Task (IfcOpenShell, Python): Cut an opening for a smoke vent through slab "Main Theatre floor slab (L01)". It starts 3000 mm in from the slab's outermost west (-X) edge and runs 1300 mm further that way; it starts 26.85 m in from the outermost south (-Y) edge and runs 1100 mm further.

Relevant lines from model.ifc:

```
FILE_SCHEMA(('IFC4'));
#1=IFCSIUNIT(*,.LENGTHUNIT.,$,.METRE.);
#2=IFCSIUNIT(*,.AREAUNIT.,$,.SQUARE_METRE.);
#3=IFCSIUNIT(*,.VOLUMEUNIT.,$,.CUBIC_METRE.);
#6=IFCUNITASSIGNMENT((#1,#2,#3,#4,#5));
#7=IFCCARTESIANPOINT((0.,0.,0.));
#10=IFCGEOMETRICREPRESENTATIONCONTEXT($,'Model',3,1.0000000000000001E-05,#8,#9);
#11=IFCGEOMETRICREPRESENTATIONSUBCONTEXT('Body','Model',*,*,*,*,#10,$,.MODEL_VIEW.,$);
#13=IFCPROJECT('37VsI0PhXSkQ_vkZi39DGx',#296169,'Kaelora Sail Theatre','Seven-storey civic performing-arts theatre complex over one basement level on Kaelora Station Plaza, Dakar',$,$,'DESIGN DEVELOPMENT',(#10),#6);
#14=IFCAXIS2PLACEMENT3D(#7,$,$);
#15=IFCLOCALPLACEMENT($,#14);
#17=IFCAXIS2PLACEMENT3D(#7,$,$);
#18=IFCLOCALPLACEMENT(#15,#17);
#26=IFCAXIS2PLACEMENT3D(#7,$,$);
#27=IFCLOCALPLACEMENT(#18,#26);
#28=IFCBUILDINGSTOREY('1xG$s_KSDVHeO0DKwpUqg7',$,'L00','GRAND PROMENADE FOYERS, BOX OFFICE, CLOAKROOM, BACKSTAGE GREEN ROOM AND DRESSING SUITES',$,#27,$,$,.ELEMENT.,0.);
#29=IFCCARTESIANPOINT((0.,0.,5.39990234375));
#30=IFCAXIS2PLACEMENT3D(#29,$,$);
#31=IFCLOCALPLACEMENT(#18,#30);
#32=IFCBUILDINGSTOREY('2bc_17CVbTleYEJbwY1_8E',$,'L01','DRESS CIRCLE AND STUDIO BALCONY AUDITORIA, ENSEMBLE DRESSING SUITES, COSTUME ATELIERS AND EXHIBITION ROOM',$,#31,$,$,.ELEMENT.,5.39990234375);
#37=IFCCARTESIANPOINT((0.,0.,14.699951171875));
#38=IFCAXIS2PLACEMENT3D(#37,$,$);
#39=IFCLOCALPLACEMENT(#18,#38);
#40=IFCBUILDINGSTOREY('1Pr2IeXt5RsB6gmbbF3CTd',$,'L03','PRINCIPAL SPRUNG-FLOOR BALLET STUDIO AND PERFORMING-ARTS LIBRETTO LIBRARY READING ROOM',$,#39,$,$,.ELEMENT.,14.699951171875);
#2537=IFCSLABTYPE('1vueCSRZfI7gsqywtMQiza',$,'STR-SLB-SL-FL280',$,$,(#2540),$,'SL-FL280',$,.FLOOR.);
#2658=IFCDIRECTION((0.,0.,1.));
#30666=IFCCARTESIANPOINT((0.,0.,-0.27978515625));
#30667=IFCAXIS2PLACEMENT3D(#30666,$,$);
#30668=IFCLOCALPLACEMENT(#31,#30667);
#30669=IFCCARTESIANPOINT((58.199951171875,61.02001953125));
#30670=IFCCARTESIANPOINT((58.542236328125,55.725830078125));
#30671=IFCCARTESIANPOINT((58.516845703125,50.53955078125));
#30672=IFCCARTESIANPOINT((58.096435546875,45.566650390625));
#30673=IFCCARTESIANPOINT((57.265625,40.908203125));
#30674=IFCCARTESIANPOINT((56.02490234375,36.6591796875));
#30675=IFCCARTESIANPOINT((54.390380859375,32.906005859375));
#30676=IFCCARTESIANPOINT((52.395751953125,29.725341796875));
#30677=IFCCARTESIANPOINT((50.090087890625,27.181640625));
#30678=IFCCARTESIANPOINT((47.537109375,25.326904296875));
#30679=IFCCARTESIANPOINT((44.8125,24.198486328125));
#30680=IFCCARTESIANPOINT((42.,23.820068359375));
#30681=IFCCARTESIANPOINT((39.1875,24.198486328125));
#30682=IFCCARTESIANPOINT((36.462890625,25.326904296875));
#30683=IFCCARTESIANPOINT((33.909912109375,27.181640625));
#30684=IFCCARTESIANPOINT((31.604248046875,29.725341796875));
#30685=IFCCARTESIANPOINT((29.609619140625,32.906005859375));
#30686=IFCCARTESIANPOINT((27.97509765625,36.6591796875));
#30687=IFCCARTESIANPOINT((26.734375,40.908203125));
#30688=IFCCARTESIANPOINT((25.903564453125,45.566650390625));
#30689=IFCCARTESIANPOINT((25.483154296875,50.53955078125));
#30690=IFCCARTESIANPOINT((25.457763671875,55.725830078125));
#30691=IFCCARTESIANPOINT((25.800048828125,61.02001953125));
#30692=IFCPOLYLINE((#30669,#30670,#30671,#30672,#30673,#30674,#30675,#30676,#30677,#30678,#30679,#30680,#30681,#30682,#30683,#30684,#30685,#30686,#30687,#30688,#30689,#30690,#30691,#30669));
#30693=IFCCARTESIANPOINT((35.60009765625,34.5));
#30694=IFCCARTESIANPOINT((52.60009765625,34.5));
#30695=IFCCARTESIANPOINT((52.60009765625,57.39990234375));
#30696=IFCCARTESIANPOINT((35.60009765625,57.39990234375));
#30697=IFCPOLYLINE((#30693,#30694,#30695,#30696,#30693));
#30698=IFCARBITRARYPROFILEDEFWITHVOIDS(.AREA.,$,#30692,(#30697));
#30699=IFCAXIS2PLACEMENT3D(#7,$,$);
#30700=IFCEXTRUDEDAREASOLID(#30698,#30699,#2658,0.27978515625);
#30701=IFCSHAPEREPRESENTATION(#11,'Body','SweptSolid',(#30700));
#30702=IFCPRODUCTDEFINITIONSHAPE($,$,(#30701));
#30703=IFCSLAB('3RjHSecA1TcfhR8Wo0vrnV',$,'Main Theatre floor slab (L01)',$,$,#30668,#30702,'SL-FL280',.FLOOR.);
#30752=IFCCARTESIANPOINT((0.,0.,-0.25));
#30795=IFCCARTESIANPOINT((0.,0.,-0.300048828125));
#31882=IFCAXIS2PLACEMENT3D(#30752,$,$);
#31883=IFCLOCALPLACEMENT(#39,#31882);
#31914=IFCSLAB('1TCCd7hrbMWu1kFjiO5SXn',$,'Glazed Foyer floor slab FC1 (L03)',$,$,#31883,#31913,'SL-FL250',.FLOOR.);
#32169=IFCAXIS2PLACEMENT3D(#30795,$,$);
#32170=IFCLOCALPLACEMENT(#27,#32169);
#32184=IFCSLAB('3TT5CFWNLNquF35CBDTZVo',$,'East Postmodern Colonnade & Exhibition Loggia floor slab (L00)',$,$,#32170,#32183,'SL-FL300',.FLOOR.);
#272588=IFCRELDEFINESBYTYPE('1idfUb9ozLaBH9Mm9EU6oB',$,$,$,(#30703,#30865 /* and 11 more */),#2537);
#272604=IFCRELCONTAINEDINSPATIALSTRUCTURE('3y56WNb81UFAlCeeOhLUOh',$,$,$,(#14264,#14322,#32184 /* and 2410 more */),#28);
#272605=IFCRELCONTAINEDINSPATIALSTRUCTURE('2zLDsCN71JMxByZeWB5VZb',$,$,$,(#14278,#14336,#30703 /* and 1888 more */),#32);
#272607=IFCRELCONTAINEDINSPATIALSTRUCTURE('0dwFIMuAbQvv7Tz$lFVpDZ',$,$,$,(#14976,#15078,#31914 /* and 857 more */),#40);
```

```python
import numpy as np
import ifcopenshell
import ifcopenshell.api.feature
import ifcopenshell.api.geometry
import ifcopenshell.api.root
import ifcopenshell.geom
import ifcopenshell.util.placement
import ifcopenshell.util.representation
import ifcopenshell.util.shape
import ifcopenshell.util.unit

model = ifcopenshell.open("model.ifc")
unit_scale = ifcopenshell.util.unit.calculate_unit_scale(model)
settings = ifcopenshell.geom.settings()


def volume(element):
    """Net volume in cubic metres, openings subtracted."""
    shape = ifcopenshell.geom.create_shape(settings, element)
    return ifcopenshell.util.shape.get_volume(shape.geometry)


slab = model.by_guid("3RjHSecA1TcfhR8Wo0vrnV")
before = volume(slab)

# Extent in the slab's own axes, in metres. The edges named are its -X and -Y sides.
slab_shape = ifcopenshell.geom.create_shape(settings, slab)
vertices = ifcopenshell.util.shape.get_vertices(slab_shape.geometry)
x_min, y_min, bottom = vertices.min(axis=0)
top = vertices[:, 2].max()

opening = ifcopenshell.api.root.create_entity(model, ifc_class="IfcOpeningElement", name="Smoke vent opening", predefined_type="OPENING")
context = ifcopenshell.util.representation.get_context(model, "Model", "Body", "MODEL_VIEW")
width, depth = 1.3, 1.1
outline = [(0.0, 0.0), (width, 0.0), (width, depth), (0.0, depth), (0.0, 0.0)]
# Overshoot both faces by 50 mm so the cut is clean.
shape = ifcopenshell.api.geometry.add_slab_representation(
    model, context=context, depth=top - bottom + 0.1, polyline=outline
)
ifcopenshell.api.geometry.assign_representation(model, product=opening, representation=shape)

matrix = ifcopenshell.util.placement.get_local_placement(slab.ObjectPlacement)
matrix[:, 3] = matrix @ np.append(np.array([x_min + 3, y_min + 26.85, bottom - 0.05]) / unit_scale, 1.0)
ifcopenshell.api.geometry.edit_object_placement(model, product=opening, matrix=matrix, is_si=False)
ifcopenshell.api.feature.add_feature(model, feature=opening, element=slab)

after = volume(slab)

print(f"slab volume {before:.3f} -> {after:.3f} m3")

model.write("model_rev.ifc")
```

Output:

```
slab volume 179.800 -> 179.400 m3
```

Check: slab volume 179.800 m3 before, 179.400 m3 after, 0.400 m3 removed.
